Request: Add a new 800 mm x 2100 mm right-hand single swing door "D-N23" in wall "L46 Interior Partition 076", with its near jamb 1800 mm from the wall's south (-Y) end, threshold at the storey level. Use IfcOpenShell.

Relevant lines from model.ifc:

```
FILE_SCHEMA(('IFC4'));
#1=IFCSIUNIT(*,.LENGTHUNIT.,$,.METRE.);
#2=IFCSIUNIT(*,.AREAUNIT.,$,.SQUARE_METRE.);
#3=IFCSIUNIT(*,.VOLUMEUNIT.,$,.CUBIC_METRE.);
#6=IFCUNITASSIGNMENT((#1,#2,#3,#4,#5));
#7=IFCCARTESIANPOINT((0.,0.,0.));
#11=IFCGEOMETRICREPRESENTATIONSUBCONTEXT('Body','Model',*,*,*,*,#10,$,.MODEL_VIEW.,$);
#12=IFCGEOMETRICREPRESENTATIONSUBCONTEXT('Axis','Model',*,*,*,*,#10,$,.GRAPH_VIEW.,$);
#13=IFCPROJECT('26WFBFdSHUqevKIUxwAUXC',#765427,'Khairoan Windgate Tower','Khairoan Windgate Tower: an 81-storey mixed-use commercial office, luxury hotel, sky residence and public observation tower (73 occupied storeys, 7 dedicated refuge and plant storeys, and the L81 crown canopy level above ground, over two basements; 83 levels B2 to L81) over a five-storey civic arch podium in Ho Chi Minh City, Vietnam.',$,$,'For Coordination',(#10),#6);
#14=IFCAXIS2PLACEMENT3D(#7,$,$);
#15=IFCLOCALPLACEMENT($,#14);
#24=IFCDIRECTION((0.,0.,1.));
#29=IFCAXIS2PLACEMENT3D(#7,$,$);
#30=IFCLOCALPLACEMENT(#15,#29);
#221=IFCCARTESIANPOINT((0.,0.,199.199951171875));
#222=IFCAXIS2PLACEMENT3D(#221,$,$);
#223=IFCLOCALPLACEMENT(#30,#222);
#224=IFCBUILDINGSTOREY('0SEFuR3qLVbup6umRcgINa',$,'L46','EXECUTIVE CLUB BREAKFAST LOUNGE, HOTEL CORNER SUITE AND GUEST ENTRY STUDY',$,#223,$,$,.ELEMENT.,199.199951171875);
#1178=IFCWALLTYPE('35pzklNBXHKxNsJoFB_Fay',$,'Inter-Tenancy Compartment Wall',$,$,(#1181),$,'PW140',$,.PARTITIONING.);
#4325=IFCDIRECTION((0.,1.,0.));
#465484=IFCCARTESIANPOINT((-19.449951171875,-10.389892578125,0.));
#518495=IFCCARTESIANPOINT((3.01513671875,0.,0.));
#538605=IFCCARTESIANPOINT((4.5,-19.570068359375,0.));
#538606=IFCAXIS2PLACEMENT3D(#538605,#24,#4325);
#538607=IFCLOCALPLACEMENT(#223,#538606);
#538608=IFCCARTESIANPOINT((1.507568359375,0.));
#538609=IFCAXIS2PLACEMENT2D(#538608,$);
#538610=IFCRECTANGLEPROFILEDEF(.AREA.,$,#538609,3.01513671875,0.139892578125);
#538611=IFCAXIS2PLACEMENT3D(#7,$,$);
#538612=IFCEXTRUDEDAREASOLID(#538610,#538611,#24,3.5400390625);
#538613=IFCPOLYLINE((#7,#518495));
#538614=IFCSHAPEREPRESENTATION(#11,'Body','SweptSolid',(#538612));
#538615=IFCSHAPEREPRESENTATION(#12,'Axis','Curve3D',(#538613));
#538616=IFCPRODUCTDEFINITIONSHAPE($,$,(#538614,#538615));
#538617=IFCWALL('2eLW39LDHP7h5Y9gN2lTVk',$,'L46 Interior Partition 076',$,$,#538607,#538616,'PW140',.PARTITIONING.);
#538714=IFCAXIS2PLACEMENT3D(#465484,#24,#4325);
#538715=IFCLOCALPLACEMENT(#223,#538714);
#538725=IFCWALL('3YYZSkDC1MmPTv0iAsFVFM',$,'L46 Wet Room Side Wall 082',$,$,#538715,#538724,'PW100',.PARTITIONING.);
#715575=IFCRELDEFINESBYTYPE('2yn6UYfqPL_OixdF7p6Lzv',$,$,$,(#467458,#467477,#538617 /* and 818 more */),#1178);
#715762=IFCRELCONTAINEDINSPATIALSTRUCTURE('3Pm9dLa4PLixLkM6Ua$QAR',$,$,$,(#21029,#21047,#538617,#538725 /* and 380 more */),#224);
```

```python
import numpy as np
import ifcopenshell
import ifcopenshell.api.feature
import ifcopenshell.api.geometry
import ifcopenshell.api.root
import ifcopenshell.api.spatial
import ifcopenshell.geom
import ifcopenshell.util.element
import ifcopenshell.util.placement
import ifcopenshell.util.representation
import ifcopenshell.util.shape
import ifcopenshell.util.unit

model = ifcopenshell.open("model.ifc")
unit_scale = ifcopenshell.util.unit.calculate_unit_scale(model)
settings = ifcopenshell.geom.settings()


def volume(element):
    """Net volume in cubic metres, openings subtracted."""
    shape = ifcopenshell.geom.create_shape(settings, element)
    return ifcopenshell.util.shape.get_volume(shape.geometry)


wall = model.by_id(538617)
storey = ifcopenshell.util.element.get_container(wall, ifc_class="IfcBuildingStorey")
context = ifcopenshell.util.representation.get_context(model, "Model", "Body", "MODEL_VIEW")
before = volume(wall)

width, height, from_end, sill = 0.8, 2.1, 1.8, 0.0  # metres

# The wall runs along its own X axis, and the end named is its -X end.
wall_shape = ifcopenshell.geom.create_shape(settings, wall)
x, y, z = ifcopenshell.util.shape.get_vertices(wall_shape.geometry).T
start = x.min() + from_end
face, thickness = float(y.min()), float(y.max() - y.min())
wall_matrix = ifcopenshell.util.placement.get_local_placement(wall.ObjectPlacement)
level = ifcopenshell.util.placement.get_local_placement(storey.ObjectPlacement)[2, 3]


def in_wall(x, y):
    """Placement at x, y metres in the wall's axes, at sill height."""
    matrix = wall_matrix.copy()
    matrix[:, 3] = wall_matrix @ np.array([x / unit_scale, y / unit_scale, 0.0, 1.0])
    matrix[2, 3] = level + sill / unit_scale
    return matrix


# Opening: a box that overshoots both wall faces by 50 mm.
opening = ifcopenshell.api.root.create_entity(model, ifc_class="IfcOpeningElement", predefined_type="OPENING")
box = ifcopenshell.api.geometry.add_wall_representation(
    model, context=context, length=width, height=height, thickness=thickness + 0.1
)
ifcopenshell.api.geometry.assign_representation(model, product=opening, representation=box)
ifcopenshell.api.geometry.edit_object_placement(model, product=opening, matrix=in_wall(start, face - 0.05), is_si=False)
ifcopenshell.api.feature.add_feature(model, feature=opening, element=wall)

door = ifcopenshell.api.root.create_entity(model, ifc_class="IfcDoor", name="D-N23", predefined_type="DOOR")
door.OverallWidth, door.OverallHeight = width / unit_scale, height / unit_scale
door.OperationType = "SINGLE_SWING_RIGHT"
body = ifcopenshell.api.geometry.add_door_representation(
    model,
    context=context,
    overall_width=door.OverallWidth,
    overall_height=door.OverallHeight,
    operation_type="SINGLE_SWING_RIGHT",
    lining_properties={"LiningDepth": thickness / unit_scale, "ThresholdDepth": thickness / unit_scale},
)
ifcopenshell.api.geometry.assign_representation(model, product=door, representation=body)
ifcopenshell.api.spatial.assign_container(model, products=[door], relating_structure=storey)
ifcopenshell.api.feature.add_filling(model, opening=opening, element=door)

# The lining spans the wall, so the door starts at the wall face.
ifcopenshell.api.geometry.edit_object_placement(model, product=door, matrix=in_wall(start, face), is_si=False)

after = volume(wall)

print(f"wall volume {before:.3f} -> {after:.3f} m3")

model.write("model_updated.ifc")
```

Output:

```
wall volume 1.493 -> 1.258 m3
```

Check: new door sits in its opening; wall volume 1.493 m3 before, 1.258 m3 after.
